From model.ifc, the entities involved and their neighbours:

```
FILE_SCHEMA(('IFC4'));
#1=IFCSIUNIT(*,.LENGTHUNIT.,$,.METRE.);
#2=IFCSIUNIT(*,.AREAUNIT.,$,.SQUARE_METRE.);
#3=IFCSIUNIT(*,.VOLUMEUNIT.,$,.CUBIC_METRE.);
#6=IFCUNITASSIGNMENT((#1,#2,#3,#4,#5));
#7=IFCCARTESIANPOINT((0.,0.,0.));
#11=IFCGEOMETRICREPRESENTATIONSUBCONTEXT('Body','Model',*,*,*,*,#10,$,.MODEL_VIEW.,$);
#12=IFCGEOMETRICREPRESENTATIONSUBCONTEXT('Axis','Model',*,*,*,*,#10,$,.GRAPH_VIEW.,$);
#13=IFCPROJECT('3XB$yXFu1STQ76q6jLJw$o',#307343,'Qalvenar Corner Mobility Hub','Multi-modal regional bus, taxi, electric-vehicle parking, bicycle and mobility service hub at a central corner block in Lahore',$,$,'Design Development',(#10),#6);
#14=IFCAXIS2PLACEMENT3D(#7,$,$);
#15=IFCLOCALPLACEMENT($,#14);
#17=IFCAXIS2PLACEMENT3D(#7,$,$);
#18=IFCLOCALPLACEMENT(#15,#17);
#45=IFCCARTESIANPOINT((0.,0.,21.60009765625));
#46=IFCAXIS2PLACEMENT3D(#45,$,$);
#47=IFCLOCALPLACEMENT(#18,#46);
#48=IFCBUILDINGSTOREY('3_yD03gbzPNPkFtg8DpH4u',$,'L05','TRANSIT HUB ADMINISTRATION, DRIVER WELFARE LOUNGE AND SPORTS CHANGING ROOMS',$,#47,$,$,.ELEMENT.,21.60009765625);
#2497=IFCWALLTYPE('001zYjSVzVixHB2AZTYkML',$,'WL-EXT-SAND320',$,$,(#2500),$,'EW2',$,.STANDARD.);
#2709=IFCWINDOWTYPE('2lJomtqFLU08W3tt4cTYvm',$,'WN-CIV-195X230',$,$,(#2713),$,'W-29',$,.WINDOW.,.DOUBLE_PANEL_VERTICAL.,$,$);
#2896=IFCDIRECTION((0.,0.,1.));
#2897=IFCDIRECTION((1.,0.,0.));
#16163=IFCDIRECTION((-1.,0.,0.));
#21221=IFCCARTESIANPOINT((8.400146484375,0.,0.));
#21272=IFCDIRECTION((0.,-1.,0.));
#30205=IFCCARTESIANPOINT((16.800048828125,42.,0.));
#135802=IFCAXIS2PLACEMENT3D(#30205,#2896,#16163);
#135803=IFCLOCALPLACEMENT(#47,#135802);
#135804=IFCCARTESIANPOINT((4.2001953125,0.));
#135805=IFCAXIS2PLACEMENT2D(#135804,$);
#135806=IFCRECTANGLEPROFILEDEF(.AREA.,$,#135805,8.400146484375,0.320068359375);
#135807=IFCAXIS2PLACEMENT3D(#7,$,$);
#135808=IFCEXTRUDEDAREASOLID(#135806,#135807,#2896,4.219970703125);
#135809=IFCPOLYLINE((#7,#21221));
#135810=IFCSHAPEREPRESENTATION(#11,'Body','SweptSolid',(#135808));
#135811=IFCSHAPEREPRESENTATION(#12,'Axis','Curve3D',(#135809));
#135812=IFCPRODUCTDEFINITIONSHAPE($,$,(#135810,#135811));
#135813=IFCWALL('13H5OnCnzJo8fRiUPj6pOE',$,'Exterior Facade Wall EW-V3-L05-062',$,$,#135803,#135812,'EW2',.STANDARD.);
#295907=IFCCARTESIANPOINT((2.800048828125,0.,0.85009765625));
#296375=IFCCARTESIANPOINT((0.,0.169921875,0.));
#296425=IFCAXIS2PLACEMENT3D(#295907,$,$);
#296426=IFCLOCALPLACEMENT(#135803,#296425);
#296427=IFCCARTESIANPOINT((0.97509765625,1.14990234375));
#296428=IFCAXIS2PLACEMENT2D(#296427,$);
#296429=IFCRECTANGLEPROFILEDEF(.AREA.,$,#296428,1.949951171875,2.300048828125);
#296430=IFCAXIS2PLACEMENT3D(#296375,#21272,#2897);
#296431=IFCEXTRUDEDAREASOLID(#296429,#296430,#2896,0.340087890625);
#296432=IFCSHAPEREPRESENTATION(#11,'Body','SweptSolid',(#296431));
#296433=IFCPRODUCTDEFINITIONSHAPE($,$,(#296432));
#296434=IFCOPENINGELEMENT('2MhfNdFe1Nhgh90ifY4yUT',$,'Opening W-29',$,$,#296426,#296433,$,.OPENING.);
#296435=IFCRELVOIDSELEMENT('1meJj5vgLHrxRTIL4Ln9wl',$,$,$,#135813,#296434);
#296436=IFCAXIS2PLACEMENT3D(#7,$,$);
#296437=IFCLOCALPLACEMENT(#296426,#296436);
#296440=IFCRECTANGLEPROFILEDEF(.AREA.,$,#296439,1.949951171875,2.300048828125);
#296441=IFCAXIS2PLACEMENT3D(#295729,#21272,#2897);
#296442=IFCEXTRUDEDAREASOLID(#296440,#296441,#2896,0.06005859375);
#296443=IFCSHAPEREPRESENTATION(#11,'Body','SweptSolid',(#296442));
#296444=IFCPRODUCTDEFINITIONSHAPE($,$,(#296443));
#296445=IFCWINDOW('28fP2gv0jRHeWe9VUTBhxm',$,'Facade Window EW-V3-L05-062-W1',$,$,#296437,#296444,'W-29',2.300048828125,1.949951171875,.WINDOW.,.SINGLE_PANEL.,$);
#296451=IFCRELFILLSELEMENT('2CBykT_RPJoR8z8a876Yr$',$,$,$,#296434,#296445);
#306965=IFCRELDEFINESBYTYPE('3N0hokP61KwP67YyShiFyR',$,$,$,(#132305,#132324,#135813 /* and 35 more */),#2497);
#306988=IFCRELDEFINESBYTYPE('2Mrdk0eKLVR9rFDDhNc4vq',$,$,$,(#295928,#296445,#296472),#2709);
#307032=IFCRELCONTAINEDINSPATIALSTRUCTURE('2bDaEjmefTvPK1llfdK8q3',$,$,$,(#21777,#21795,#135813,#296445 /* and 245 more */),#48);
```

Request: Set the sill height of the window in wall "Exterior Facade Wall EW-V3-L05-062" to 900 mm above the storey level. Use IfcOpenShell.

```python
import numpy as np
import ifcopenshell
import ifcopenshell.api.geometry
import ifcopenshell.geom
import ifcopenshell.util.element
import ifcopenshell.util.placement
import ifcopenshell.util.shape
import ifcopenshell.util.unit

model = ifcopenshell.open("model.ifc")
unit_scale = ifcopenshell.util.unit.calculate_unit_scale(model)

window = model.by_guid("28fP2gv0jRHeWe9VUTBhxm")
opening = window.FillsVoids[0].RelatingOpeningElement
storey = ifcopenshell.util.element.get_container(window, ifc_class="IfcBuildingStorey")
level = ifcopenshell.util.placement.get_local_placement(storey.ObjectPlacement)[2, 3]

# The opening's origin need not be at the sill, so measure its lowest point.
shape = ifcopenshell.geom.create_shape(ifcopenshell.geom.settings(), opening)
bottom = ifcopenshell.util.shape.get_shape_bottom_elevation(shape, shape.geometry) / unit_scale
dz = level + 0.9 / unit_scale - bottom

shift = np.array([0.0, 0.0, dz])
# The window is placed relative to its opening, so it follows when the opening moves.
matrix = ifcopenshell.util.placement.get_local_placement(opening.ObjectPlacement)
matrix[:3, 3] += shift
ifcopenshell.api.geometry.edit_object_placement(
    model, product=opening, matrix=matrix, is_si=False, should_transform_children=True
)

print(f"moved by {dz * unit_scale:+.3f} m")

model.write("model_edited.ifc")
```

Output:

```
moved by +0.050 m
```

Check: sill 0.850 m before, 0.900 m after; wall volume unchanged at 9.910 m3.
